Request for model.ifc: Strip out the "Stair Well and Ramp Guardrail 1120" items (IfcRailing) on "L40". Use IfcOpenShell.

First a look at what the model holds.

```python
import ifcopenshell
import ifcopenshell.util.element

model = ifcopenshell.open("model.ifc")
print(model.schema)
storey = next(s for s in model.by_type("IfcBuildingStorey") if s.Name == "L40")
railings = [e for e in ifcopenshell.util.element.get_decomposition(storey) if e.is_a("IfcRailing")]
seen = {}
for e in railings:
    element_type = ifcopenshell.util.element.get_type(e)
    name = element_type.Name if element_type not in (None, e) else None
    seen[name] = seen.get(name, 0) + 1
for name, count in sorted(seen.items(), key=str):
    print(count, "x", name)
```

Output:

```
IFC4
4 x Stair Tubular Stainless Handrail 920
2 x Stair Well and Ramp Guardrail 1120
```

```python
import ifcopenshell
import ifcopenshell.api.root
import ifcopenshell.util.element

model = ifcopenshell.open("model.ifc")

storey = next(s for s in model.by_type("IfcBuildingStorey") if s.Name == "L40")
railings = [e for e in ifcopenshell.util.element.get_decomposition(storey) if e.is_a("IfcRailing")]
targets = [e for e in railings if (t := ifcopenshell.util.element.get_type(e)) not in (None, e) and t.Name == "Stair Well and Ramp Guardrail 1120"]

for e in targets:
    ifcopenshell.api.root.remove_product(model, product=e)
print(len(targets), "removed")

model.write("model_updated.ifc")
```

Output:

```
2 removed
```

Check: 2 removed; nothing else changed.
